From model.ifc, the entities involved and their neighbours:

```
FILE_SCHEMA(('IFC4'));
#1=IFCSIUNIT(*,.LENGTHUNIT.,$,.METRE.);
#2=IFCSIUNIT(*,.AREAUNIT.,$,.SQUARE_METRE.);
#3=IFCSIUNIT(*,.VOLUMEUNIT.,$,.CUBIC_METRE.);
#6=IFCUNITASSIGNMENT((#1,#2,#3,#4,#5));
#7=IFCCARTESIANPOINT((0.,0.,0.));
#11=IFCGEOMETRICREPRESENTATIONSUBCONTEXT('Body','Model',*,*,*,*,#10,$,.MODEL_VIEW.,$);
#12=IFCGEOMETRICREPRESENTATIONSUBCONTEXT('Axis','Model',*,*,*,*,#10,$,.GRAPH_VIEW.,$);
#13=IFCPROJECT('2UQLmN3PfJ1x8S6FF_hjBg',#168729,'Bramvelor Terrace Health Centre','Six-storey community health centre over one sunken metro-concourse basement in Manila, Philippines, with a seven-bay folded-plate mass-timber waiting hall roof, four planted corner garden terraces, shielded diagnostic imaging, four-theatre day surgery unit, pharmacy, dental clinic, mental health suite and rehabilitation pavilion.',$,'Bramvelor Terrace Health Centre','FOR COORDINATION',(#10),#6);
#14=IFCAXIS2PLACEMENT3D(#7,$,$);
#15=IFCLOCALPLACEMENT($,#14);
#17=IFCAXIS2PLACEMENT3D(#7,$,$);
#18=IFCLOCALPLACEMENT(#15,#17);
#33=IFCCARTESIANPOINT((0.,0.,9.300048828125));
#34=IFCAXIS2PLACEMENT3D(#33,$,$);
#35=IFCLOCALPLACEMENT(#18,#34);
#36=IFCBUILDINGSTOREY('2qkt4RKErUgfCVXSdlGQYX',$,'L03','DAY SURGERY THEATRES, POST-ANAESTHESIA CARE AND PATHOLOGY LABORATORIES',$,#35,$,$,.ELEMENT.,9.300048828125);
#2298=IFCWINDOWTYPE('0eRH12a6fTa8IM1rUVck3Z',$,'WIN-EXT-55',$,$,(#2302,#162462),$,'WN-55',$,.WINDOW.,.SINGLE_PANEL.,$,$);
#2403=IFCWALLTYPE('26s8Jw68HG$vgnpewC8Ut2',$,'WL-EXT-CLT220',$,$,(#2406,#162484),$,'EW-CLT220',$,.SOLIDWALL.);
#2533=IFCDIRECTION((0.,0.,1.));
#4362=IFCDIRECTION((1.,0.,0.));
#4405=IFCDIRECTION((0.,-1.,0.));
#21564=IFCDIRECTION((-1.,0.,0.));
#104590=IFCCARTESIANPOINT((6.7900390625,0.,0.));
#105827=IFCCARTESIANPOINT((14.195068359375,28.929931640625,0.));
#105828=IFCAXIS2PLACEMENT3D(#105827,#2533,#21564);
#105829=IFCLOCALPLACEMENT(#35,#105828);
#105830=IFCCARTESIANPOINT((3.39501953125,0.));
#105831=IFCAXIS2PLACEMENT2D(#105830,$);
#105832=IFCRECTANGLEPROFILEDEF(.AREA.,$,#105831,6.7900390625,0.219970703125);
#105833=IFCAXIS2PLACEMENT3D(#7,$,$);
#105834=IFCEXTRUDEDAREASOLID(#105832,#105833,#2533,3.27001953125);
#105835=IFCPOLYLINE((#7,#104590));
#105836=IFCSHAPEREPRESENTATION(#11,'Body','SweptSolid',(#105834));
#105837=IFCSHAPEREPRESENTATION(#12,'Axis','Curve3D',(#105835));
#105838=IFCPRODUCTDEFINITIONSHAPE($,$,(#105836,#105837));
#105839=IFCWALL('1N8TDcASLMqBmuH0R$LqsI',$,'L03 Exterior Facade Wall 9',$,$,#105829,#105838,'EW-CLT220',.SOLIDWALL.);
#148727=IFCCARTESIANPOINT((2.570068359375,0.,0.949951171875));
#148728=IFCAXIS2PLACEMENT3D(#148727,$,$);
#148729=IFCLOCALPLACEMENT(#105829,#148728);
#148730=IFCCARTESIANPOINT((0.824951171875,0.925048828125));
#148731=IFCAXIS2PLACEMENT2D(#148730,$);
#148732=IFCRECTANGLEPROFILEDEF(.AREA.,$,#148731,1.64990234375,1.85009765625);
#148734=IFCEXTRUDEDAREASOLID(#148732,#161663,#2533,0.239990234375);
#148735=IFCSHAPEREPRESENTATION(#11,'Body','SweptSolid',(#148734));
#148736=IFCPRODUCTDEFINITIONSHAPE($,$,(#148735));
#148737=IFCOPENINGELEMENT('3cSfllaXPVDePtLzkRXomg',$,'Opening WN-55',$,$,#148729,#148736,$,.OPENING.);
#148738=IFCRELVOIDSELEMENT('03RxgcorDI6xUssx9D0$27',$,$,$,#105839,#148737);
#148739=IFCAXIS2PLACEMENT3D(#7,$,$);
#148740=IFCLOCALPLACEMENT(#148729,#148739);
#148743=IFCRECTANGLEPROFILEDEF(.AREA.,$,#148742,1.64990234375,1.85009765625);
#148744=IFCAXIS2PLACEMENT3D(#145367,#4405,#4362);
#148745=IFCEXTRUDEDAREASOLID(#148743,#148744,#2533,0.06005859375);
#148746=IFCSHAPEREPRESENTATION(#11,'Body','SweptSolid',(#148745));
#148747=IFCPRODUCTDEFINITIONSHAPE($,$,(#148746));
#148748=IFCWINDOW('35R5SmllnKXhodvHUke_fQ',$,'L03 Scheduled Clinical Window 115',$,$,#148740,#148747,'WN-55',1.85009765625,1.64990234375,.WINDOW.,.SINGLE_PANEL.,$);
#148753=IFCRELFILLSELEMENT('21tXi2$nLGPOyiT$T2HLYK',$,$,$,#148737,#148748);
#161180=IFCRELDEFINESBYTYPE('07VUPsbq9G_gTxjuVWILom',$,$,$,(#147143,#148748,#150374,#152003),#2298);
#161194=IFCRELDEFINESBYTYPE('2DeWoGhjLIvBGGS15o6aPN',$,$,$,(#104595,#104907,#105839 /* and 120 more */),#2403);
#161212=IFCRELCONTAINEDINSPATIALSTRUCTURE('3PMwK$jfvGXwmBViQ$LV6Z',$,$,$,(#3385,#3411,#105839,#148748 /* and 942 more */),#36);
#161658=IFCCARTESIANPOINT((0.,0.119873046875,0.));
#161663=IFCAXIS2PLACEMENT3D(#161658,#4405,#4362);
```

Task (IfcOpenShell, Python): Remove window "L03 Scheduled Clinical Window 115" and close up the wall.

```python
import ifcopenshell
import ifcopenshell.api.feature
import ifcopenshell.api.root
import ifcopenshell.geom
import ifcopenshell.util.shape

model = ifcopenshell.open("model.ifc")
settings = ifcopenshell.geom.settings()


def volume(element):
    """Net volume in cubic metres, openings subtracted."""
    shape = ifcopenshell.geom.create_shape(settings, element)
    return ifcopenshell.util.shape.get_volume(shape.geometry)


window = model.by_id(148748)
opening = window.FillsVoids[0].RelatingOpeningElement
wall = opening.VoidsElements[0].RelatingBuildingElement
before = volume(wall)

ifcopenshell.api.root.remove_product(model, product=window)
ifcopenshell.api.feature.remove_feature(model, feature=opening)

after = volume(wall)

print(f"wall volume {before:.3f} -> {after:.3f} m3")

model.write("model_edited.ifc")
```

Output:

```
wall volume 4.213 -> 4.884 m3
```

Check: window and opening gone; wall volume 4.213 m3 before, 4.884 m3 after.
